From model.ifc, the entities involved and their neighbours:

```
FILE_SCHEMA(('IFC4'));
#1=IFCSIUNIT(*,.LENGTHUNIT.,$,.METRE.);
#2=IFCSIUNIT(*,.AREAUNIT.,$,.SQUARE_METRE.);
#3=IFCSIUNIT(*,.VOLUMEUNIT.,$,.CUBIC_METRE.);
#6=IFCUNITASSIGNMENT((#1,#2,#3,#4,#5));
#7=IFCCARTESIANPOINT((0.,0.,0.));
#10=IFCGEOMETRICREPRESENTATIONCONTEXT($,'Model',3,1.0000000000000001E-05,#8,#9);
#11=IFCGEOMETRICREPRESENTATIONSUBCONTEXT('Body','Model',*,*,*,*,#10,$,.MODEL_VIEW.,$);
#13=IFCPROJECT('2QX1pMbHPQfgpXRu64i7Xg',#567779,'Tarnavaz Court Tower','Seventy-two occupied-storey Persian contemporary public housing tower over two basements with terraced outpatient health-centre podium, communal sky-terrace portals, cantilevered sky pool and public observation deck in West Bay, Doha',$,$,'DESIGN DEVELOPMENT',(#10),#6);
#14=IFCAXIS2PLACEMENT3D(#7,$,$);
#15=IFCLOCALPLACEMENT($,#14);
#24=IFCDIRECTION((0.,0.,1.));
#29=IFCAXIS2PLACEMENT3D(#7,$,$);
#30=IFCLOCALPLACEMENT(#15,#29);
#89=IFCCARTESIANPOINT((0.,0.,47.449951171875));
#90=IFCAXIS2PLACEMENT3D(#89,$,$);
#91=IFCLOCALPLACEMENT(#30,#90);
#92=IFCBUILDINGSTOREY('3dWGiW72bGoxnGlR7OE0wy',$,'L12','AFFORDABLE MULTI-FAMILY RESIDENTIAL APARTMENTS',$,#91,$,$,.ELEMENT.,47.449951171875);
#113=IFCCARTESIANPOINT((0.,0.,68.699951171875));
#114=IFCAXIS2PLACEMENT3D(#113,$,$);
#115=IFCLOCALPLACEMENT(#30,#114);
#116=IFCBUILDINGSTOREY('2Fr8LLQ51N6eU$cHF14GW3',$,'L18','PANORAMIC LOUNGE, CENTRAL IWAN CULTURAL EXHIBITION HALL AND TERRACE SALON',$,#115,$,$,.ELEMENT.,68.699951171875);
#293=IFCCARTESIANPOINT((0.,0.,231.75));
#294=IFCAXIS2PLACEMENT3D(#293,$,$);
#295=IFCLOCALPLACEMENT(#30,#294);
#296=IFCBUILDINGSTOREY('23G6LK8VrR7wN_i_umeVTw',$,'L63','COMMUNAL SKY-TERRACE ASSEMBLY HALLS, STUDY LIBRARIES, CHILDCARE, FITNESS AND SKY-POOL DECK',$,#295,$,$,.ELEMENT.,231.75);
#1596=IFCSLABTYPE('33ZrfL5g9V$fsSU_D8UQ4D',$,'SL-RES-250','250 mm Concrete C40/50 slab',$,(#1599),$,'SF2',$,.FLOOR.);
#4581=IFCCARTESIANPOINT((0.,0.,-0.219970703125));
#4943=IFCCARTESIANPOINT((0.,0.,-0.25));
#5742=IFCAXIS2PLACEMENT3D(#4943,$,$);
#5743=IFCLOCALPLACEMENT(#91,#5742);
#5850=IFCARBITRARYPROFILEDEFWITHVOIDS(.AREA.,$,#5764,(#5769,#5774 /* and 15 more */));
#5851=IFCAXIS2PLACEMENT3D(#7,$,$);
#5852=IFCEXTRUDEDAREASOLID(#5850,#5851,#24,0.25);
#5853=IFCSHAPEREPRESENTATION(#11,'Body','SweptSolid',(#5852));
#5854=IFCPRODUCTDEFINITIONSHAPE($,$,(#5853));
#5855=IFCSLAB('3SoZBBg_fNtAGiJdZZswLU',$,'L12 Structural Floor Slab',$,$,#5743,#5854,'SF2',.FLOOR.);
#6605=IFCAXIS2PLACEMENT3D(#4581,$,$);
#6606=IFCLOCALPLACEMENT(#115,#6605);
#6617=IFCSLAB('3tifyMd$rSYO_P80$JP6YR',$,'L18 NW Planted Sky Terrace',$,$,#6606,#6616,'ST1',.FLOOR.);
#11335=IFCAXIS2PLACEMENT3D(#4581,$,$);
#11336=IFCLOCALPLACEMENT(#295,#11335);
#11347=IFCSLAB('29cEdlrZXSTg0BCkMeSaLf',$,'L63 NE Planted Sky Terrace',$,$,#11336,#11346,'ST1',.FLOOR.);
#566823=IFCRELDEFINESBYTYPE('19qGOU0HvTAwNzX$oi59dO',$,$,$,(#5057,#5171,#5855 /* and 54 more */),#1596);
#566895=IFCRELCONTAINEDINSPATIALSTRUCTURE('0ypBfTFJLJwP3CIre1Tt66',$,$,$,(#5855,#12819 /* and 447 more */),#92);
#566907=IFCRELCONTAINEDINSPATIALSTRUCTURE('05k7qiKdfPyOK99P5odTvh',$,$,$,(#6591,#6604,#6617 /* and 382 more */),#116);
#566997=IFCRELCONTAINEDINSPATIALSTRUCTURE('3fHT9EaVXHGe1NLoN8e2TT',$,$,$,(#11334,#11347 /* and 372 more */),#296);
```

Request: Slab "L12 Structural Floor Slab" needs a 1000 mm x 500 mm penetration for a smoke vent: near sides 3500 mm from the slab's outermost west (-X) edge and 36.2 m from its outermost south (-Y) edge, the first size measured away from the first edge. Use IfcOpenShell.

```python
import numpy as np
import ifcopenshell
import ifcopenshell.api.feature
import ifcopenshell.api.geometry
import ifcopenshell.api.root
import ifcopenshell.geom
import ifcopenshell.util.placement
import ifcopenshell.util.representation
import ifcopenshell.util.shape
import ifcopenshell.util.unit

model = ifcopenshell.open("model.ifc")
unit_scale = ifcopenshell.util.unit.calculate_unit_scale(model)
settings = ifcopenshell.geom.settings()


def volume(element):
    """Net volume in cubic metres, openings subtracted."""
    shape = ifcopenshell.geom.create_shape(settings, element)
    return ifcopenshell.util.shape.get_volume(shape.geometry)


slab = model.by_guid("3SoZBBg_fNtAGiJdZZswLU")
before = volume(slab)

# Extent in the slab's own axes, in metres. The edges named are its -X and -Y sides.
slab_shape = ifcopenshell.geom.create_shape(settings, slab)
vertices = ifcopenshell.util.shape.get_vertices(slab_shape.geometry)
x_min, y_min, bottom = vertices.min(axis=0)
top = vertices[:, 2].max()

opening = ifcopenshell.api.root.create_entity(model, ifc_class="IfcOpeningElement", name="Smoke vent opening", predefined_type="OPENING")
context = ifcopenshell.util.representation.get_context(model, "Model", "Body", "MODEL_VIEW")
width, depth = 1, 0.5
outline = [(0.0, 0.0), (width, 0.0), (width, depth), (0.0, depth), (0.0, 0.0)]
# Overshoot both faces by 50 mm so the cut is clean.
shape = ifcopenshell.api.geometry.add_slab_representation(
    model, context=context, depth=top - bottom + 0.1, polyline=outline
)
ifcopenshell.api.geometry.assign_representation(model, product=opening, representation=shape)

matrix = ifcopenshell.util.placement.get_local_placement(slab.ObjectPlacement)
matrix[:, 3] = matrix @ np.append(np.array([x_min + 3.5, y_min + 36.2, bottom - 0.05]) / unit_scale, 1.0)
ifcopenshell.api.geometry.edit_object_placement(model, product=opening, matrix=matrix, is_si=False)
ifcopenshell.api.feature.add_feature(model, feature=opening, element=slab)

after = volume(slab)

print(f"slab volume {before:.3f} -> {after:.3f} m3")

model.write("model_updated.ifc")
```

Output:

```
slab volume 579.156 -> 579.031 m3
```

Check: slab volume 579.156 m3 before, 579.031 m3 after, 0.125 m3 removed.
